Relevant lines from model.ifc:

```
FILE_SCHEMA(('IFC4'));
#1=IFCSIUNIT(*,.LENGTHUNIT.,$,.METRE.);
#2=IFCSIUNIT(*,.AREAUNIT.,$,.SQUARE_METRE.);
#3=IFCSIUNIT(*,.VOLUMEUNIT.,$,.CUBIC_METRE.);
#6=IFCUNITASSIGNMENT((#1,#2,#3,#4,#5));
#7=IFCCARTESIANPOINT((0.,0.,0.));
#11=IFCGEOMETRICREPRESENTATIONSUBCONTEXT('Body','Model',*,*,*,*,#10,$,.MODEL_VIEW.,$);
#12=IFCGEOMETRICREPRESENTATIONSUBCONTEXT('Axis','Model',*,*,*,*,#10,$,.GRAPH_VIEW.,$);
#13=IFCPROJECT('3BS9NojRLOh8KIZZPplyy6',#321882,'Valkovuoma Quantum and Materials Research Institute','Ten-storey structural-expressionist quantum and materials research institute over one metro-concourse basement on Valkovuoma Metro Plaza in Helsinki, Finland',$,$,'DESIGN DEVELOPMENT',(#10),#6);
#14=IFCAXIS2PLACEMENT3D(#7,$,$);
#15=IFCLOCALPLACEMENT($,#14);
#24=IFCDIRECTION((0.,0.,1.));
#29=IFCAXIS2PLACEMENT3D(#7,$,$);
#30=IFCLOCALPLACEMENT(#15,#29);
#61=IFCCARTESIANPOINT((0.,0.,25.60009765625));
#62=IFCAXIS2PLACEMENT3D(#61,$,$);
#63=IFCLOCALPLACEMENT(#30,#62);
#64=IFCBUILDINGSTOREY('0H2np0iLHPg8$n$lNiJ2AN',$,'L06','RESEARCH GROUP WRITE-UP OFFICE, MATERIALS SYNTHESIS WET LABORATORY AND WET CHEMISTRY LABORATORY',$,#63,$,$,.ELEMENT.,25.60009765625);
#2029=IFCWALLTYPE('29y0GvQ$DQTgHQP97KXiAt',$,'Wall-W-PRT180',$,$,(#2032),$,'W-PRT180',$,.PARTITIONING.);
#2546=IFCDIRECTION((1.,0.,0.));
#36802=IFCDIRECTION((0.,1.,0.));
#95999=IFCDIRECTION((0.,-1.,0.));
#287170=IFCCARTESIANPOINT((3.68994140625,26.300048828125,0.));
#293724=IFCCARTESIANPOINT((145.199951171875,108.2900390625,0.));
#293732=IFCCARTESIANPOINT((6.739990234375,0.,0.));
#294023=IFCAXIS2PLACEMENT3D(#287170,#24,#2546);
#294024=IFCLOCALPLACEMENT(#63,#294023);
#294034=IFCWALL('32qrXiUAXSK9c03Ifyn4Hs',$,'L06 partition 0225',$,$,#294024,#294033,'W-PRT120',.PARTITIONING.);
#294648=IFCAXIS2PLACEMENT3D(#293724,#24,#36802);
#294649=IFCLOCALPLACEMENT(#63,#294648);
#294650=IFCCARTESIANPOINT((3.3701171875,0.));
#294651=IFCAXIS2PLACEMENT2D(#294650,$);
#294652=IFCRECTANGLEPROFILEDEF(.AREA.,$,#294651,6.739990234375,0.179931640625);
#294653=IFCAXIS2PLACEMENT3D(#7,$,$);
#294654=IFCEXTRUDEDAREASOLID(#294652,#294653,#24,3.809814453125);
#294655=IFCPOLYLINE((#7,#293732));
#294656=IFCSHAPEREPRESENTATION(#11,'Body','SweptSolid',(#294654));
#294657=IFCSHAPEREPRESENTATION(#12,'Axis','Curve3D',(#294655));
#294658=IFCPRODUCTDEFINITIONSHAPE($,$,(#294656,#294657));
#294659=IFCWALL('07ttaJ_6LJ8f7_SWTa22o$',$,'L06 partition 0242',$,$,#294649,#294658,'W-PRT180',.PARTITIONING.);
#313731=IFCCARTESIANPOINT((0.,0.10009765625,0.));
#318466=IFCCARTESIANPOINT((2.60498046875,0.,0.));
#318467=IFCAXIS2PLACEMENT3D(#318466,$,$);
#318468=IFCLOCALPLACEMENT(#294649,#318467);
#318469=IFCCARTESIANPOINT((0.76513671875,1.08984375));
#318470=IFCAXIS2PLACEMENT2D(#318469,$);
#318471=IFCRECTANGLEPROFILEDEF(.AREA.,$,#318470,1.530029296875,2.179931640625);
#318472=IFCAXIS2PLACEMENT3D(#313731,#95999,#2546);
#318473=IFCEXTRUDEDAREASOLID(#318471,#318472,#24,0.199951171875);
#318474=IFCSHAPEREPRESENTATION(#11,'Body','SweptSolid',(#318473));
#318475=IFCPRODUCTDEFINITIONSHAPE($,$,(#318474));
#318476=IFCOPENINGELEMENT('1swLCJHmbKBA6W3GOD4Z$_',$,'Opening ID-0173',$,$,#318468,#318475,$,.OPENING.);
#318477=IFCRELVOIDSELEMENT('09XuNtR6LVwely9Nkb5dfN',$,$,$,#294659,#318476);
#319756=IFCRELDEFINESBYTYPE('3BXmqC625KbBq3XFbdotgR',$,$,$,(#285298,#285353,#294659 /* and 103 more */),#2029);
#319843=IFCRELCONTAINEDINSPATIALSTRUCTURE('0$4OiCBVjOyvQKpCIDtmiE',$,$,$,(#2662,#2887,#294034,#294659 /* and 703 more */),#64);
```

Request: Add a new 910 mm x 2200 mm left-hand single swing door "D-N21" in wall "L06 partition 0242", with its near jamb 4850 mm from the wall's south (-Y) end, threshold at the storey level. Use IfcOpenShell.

```python
import numpy as np
import ifcopenshell
import ifcopenshell.api.feature
import ifcopenshell.api.geometry
import ifcopenshell.api.root
import ifcopenshell.api.spatial
import ifcopenshell.geom
import ifcopenshell.util.element
import ifcopenshell.util.placement
import ifcopenshell.util.representation
import ifcopenshell.util.shape
import ifcopenshell.util.unit

model = ifcopenshell.open("model.ifc")
unit_scale = ifcopenshell.util.unit.calculate_unit_scale(model)
settings = ifcopenshell.geom.settings()


def volume(element):
    """Net volume in cubic metres, openings subtracted."""
    shape = ifcopenshell.geom.create_shape(settings, element)
    return ifcopenshell.util.shape.get_volume(shape.geometry)


wall = model.by_guid("07ttaJ_6LJ8f7_SWTa22o$")
storey = ifcopenshell.util.element.get_container(wall, ifc_class="IfcBuildingStorey")
context = ifcopenshell.util.representation.get_context(model, "Model", "Body", "MODEL_VIEW")
before = volume(wall)

width, height, from_end, sill = 0.91, 2.2, 4.85, 0.0  # metres

# The wall runs along its own X axis, and the end named is its -X end.
wall_shape = ifcopenshell.geom.create_shape(settings, wall)
x, y, z = ifcopenshell.util.shape.get_vertices(wall_shape.geometry).T
start = x.min() + from_end
face, thickness = float(y.min()), float(y.max() - y.min())
wall_matrix = ifcopenshell.util.placement.get_local_placement(wall.ObjectPlacement)
level = ifcopenshell.util.placement.get_local_placement(storey.ObjectPlacement)[2, 3]


def in_wall(x, y):
    """Placement at x, y metres in the wall's axes, at sill height."""
    matrix = wall_matrix.copy()
    matrix[:, 3] = wall_matrix @ np.array([x / unit_scale, y / unit_scale, 0.0, 1.0])
    matrix[2, 3] = level + sill / unit_scale
    return matrix


# Opening: a box that overshoots both wall faces by 50 mm.
opening = ifcopenshell.api.root.create_entity(model, ifc_class="IfcOpeningElement", predefined_type="OPENING")
box = ifcopenshell.api.geometry.add_wall_representation(
    model, context=context, length=width, height=height, thickness=thickness + 0.1
)
ifcopenshell.api.geometry.assign_representation(model, product=opening, representation=box)
ifcopenshell.api.geometry.edit_object_placement(model, product=opening, matrix=in_wall(start, face - 0.05), is_si=False)
ifcopenshell.api.feature.add_feature(model, feature=opening, element=wall)

door = ifcopenshell.api.root.create_entity(model, ifc_class="IfcDoor", name="D-N21", predefined_type="DOOR")
door.OverallWidth, door.OverallHeight = width / unit_scale, height / unit_scale
door.OperationType = "SINGLE_SWING_LEFT"
body = ifcopenshell.api.geometry.add_door_representation(
    model,
    context=context,
    overall_width=door.OverallWidth,
    overall_height=door.OverallHeight,
    operation_type="SINGLE_SWING_LEFT",
    lining_properties={"LiningDepth": thickness / unit_scale, "ThresholdDepth": thickness / unit_scale},
)
ifcopenshell.api.geometry.assign_representation(model, product=door, representation=body)
ifcopenshell.api.spatial.assign_container(model, products=[door], relating_structure=storey)
ifcopenshell.api.feature.add_filling(model, opening=opening, element=door)

# The lining spans the wall, so the door starts at the wall face.
ifcopenshell.api.geometry.edit_object_placement(model, product=door, matrix=in_wall(start, face), is_si=False)

after = volume(wall)

print(f"wall volume {before:.3f} -> {after:.3f} m3")

model.write("model_edited.ifc")
```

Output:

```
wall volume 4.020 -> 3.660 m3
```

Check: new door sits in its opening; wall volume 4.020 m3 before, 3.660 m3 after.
